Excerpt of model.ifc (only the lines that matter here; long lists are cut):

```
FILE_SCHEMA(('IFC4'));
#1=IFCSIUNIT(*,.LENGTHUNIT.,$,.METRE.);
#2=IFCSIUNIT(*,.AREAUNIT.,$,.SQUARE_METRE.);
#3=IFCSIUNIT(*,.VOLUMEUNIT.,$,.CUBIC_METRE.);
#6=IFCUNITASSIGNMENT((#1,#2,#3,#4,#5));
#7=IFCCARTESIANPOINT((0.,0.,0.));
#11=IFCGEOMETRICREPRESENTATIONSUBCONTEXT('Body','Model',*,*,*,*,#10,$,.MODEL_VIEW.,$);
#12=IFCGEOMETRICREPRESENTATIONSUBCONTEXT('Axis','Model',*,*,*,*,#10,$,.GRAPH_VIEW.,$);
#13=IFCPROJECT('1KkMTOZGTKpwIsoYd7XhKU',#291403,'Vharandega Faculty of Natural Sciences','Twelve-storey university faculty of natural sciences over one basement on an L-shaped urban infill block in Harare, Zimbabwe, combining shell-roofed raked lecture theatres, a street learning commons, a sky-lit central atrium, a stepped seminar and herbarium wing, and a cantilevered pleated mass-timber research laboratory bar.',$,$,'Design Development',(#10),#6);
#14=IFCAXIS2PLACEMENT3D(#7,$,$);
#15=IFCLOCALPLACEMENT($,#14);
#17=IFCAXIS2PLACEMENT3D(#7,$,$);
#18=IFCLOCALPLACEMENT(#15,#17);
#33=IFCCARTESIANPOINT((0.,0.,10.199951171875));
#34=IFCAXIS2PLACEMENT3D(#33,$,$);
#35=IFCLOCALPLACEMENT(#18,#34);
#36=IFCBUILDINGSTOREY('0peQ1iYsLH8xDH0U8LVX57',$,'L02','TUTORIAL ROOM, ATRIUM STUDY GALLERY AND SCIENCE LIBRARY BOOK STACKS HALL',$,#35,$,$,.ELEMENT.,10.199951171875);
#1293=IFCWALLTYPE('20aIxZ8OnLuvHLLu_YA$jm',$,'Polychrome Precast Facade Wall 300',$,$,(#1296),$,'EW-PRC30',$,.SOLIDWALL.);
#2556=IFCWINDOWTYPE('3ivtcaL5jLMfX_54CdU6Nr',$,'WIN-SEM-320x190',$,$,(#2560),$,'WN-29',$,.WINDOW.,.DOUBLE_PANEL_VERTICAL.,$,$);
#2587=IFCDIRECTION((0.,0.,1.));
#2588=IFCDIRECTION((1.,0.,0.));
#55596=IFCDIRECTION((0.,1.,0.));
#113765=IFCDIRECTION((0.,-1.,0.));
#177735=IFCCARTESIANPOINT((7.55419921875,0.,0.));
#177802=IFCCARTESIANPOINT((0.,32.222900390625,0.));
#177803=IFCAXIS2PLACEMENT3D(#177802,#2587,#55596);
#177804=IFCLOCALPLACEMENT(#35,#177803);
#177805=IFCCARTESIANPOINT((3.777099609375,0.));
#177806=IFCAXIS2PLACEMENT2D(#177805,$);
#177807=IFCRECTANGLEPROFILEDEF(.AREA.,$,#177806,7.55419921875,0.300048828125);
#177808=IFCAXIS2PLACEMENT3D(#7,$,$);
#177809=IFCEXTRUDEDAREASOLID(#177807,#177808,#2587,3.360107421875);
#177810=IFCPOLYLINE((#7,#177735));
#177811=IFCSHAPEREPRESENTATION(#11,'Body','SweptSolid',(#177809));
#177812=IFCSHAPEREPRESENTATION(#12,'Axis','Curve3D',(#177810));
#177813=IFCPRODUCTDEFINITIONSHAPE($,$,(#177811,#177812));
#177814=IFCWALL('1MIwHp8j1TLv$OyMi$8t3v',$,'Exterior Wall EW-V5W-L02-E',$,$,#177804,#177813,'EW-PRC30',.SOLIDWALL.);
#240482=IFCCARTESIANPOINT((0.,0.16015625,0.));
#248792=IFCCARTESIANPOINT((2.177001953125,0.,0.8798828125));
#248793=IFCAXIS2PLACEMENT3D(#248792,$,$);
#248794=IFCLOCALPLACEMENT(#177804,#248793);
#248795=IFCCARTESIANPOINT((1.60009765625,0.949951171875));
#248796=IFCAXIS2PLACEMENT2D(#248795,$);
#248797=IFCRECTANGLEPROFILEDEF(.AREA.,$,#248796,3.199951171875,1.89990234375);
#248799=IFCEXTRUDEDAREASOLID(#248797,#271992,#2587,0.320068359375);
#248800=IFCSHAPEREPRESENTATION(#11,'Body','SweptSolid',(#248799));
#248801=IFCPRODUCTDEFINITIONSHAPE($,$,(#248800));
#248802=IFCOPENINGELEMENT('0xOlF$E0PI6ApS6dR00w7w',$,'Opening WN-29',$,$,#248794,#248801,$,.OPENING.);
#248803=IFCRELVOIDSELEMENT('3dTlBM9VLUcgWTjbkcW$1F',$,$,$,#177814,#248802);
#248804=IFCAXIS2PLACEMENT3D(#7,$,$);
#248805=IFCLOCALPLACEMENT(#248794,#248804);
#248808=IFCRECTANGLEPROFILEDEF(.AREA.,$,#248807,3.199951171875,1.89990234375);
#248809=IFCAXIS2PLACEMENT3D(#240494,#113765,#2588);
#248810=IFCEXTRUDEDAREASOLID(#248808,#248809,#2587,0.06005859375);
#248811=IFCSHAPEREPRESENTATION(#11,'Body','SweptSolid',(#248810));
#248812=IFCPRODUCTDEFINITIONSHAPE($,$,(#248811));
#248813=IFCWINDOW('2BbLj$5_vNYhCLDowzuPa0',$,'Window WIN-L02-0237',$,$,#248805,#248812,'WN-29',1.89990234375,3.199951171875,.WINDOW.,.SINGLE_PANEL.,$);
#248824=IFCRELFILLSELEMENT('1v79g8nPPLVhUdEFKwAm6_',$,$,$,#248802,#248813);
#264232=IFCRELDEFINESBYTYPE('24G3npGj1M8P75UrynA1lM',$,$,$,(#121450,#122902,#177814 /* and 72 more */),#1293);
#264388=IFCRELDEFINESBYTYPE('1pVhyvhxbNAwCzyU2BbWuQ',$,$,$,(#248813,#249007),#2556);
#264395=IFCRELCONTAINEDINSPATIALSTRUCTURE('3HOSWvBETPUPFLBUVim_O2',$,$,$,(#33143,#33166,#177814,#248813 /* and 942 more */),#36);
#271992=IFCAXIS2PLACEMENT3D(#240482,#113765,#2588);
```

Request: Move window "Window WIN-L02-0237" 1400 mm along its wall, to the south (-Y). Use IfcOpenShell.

```python
import ifcopenshell
import ifcopenshell.api.geometry
import ifcopenshell.util.placement
import ifcopenshell.util.unit

model = ifcopenshell.open("model.ifc")
unit_scale = ifcopenshell.util.unit.calculate_unit_scale(model)

window = model.by_guid("2BbLj$5_vNYhCLDowzuPa0")
opening = window.FillsVoids[0].RelatingOpeningElement
wall = opening.VoidsElements[0].RelatingBuildingElement

wall_matrix = ifcopenshell.util.placement.get_local_placement(wall.ObjectPlacement)
shift = wall_matrix[:3, 0] * -1.4 / unit_scale
before = ifcopenshell.util.placement.get_local_placement(window.ObjectPlacement)[:3, 3].copy()

# The window is placed relative to its opening, so it follows when the opening moves.
matrix = ifcopenshell.util.placement.get_local_placement(opening.ObjectPlacement)
matrix[:3, 3] += shift
ifcopenshell.api.geometry.edit_object_placement(
    model, product=opening, matrix=matrix, is_si=False, should_transform_children=True
)

after = ifcopenshell.util.placement.get_local_placement(window.ObjectPlacement)[:3, 3]
print("window moved by", (after - before).round(3) + 0.0)

model.write("model_edited.ifc")
```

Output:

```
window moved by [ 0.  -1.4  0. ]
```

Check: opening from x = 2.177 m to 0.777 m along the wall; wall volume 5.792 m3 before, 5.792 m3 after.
